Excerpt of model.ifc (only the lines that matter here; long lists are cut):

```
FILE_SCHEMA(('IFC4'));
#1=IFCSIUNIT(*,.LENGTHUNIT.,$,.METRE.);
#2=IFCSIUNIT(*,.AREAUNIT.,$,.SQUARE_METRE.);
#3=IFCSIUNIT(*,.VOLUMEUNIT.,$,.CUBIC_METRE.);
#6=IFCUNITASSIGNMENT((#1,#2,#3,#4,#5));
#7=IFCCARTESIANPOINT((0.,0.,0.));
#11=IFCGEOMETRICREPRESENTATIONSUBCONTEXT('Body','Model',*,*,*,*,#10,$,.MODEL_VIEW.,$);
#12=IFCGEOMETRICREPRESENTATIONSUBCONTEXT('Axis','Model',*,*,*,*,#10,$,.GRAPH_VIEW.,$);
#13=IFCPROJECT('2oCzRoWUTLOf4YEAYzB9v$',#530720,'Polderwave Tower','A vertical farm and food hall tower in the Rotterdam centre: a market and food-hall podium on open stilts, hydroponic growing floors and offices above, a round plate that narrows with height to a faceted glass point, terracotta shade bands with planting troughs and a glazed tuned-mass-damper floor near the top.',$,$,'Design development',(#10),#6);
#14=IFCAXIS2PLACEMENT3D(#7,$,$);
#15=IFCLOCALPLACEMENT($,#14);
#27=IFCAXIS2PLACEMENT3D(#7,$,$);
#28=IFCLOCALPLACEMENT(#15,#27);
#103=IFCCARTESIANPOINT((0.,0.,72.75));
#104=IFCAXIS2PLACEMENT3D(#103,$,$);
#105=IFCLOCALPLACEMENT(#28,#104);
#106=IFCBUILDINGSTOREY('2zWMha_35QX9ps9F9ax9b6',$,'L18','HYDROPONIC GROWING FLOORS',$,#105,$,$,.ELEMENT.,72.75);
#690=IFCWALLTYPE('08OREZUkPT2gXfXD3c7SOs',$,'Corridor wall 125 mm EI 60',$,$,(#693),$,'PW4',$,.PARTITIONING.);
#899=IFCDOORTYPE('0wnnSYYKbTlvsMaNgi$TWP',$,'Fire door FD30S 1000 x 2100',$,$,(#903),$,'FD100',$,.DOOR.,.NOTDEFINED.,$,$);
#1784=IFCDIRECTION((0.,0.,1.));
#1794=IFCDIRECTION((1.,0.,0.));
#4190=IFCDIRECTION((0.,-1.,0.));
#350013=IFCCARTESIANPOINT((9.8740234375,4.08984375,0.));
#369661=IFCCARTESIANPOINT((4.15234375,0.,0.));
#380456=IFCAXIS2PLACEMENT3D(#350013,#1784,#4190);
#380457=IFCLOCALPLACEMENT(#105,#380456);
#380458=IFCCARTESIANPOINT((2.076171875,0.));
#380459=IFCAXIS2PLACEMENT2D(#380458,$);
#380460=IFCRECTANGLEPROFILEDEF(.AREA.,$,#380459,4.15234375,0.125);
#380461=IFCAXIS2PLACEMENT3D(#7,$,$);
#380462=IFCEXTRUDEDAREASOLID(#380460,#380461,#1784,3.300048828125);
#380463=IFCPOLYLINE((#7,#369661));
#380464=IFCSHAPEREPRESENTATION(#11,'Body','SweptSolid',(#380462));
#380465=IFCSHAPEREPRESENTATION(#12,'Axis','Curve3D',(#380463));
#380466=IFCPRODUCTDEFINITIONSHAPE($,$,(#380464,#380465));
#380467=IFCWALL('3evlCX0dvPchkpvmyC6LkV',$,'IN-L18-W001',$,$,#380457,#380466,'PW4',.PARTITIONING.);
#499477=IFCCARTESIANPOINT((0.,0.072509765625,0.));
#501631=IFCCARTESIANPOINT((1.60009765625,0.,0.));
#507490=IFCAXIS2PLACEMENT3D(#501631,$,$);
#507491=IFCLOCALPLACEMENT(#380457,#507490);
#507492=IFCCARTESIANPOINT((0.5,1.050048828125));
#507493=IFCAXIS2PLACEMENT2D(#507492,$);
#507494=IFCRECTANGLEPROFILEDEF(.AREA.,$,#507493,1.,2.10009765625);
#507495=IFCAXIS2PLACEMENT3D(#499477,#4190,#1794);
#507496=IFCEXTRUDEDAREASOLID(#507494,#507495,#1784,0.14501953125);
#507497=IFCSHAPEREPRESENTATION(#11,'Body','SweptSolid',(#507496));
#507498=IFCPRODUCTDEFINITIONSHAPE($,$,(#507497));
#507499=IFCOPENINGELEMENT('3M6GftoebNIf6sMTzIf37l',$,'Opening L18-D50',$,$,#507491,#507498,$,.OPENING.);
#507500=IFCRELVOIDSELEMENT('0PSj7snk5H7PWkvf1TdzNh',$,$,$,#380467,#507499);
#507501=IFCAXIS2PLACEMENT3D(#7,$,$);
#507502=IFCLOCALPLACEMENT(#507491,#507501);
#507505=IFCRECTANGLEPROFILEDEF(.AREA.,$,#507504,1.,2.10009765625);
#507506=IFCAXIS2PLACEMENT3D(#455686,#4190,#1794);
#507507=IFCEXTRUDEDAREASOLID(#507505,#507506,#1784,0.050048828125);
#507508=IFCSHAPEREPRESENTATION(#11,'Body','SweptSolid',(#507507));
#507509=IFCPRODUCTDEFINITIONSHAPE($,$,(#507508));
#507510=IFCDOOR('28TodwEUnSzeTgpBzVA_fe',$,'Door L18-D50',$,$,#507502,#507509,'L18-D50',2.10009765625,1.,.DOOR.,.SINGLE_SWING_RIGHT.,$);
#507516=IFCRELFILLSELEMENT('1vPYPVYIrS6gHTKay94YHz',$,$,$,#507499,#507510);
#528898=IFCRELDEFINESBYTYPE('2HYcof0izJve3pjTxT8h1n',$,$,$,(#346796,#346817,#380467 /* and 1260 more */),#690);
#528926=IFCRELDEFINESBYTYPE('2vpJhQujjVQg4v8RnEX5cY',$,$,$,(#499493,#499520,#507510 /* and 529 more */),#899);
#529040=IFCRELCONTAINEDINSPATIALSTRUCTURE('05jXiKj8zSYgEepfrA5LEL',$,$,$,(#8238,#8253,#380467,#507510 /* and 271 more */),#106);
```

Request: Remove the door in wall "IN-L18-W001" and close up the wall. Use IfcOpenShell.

```python
import ifcopenshell
import ifcopenshell.api.feature
import ifcopenshell.api.root
import ifcopenshell.geom
import ifcopenshell.util.shape

model = ifcopenshell.open("model.ifc")
settings = ifcopenshell.geom.settings()


def volume(element):
    """Net volume in cubic metres, openings subtracted."""
    shape = ifcopenshell.geom.create_shape(settings, element)
    return ifcopenshell.util.shape.get_volume(shape.geometry)


door = model.by_guid("28TodwEUnSzeTgpBzVA_fe")
opening = door.FillsVoids[0].RelatingOpeningElement
wall = opening.VoidsElements[0].RelatingBuildingElement
before = volume(wall)

ifcopenshell.api.root.remove_product(model, product=door)
ifcopenshell.api.feature.remove_feature(model, feature=opening)

after = volume(wall)

print(f"wall volume {before:.3f} -> {after:.3f} m3")

model.write("model_edited.ifc")
```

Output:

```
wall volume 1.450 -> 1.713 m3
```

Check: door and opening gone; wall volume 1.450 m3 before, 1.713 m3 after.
